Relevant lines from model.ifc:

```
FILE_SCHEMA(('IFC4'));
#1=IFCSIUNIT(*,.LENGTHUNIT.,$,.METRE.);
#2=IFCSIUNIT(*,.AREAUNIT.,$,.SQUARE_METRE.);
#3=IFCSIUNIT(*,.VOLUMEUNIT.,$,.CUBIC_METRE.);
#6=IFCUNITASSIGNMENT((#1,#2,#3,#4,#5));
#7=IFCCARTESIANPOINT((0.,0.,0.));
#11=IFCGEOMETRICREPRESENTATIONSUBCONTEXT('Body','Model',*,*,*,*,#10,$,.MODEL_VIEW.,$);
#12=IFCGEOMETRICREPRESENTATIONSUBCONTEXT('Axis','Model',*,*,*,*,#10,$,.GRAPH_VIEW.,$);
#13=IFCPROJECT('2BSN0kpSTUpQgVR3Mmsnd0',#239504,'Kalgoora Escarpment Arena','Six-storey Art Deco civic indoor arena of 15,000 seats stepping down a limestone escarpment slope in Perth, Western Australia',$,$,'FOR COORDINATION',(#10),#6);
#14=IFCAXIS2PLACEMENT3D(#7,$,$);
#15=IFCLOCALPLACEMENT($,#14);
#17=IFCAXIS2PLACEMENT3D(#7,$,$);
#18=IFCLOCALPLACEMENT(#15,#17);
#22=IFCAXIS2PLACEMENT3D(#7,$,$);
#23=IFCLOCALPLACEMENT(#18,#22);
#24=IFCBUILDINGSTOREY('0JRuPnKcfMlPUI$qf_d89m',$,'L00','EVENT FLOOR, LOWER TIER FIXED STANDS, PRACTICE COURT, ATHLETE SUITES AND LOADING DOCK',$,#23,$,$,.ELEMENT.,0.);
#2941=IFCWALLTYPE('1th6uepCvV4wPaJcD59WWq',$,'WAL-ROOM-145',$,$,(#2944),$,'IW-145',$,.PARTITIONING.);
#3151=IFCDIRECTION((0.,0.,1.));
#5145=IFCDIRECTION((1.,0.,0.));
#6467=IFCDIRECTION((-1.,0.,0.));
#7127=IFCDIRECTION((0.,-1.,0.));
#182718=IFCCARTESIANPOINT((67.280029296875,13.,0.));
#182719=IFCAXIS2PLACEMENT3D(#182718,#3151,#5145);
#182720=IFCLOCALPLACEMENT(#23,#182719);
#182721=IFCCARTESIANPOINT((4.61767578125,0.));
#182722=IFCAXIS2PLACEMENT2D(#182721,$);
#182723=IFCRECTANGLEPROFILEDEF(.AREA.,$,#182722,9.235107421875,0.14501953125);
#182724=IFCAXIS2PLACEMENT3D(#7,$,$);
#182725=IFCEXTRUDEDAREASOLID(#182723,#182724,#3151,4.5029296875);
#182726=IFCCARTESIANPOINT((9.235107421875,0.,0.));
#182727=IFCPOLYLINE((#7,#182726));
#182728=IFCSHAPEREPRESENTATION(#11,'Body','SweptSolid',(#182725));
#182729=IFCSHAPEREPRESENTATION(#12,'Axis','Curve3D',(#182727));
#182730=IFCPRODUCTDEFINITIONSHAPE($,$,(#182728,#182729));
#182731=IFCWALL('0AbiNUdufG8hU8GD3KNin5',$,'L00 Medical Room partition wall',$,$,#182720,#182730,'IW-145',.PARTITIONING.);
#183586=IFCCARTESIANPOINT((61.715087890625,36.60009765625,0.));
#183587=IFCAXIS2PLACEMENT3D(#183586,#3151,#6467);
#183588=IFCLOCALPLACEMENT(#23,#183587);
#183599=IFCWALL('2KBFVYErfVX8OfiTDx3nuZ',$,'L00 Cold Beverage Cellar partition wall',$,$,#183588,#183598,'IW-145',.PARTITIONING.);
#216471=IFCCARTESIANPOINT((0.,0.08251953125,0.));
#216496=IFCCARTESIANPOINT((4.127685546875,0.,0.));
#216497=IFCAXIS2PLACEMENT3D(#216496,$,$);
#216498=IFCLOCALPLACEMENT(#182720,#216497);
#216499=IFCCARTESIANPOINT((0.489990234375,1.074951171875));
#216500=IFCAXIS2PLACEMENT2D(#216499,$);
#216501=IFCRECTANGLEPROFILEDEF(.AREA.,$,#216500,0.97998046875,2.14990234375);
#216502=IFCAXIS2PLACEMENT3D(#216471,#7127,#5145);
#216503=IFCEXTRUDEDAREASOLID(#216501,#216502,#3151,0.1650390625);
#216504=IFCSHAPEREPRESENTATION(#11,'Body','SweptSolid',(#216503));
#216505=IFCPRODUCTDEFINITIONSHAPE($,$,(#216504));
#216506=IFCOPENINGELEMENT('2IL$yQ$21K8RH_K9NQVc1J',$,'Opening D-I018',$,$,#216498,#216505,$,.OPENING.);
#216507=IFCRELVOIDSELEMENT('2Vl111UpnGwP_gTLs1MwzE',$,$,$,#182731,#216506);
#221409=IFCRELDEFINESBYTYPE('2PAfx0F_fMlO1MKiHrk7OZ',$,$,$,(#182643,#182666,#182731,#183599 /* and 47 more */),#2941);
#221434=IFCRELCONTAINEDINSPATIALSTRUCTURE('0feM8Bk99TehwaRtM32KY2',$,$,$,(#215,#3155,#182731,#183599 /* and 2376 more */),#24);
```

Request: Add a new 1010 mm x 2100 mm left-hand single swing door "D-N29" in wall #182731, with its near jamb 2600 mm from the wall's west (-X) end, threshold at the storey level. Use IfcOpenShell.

```python
import numpy as np
import ifcopenshell
import ifcopenshell.api.feature
import ifcopenshell.api.geometry
import ifcopenshell.api.root
import ifcopenshell.api.spatial
import ifcopenshell.geom
import ifcopenshell.util.element
import ifcopenshell.util.placement
import ifcopenshell.util.representation
import ifcopenshell.util.shape
import ifcopenshell.util.unit

model = ifcopenshell.open("model.ifc")
unit_scale = ifcopenshell.util.unit.calculate_unit_scale(model)
settings = ifcopenshell.geom.settings()


def volume(element):
    """Net volume in cubic metres, openings subtracted."""
    shape = ifcopenshell.geom.create_shape(settings, element)
    return ifcopenshell.util.shape.get_volume(shape.geometry)


wall = model.by_guid("0AbiNUdufG8hU8GD3KNin5")
storey = ifcopenshell.util.element.get_container(wall, ifc_class="IfcBuildingStorey")
context = ifcopenshell.util.representation.get_context(model, "Model", "Body", "MODEL_VIEW")
before = volume(wall)

width, height, from_end, sill = 1.01, 2.1, 2.6, 0.0  # metres

# The wall runs along its own X axis, and the end named is its -X end.
wall_shape = ifcopenshell.geom.create_shape(settings, wall)
x, y, z = ifcopenshell.util.shape.get_vertices(wall_shape.geometry).T
start = x.min() + from_end
face, thickness = float(y.min()), float(y.max() - y.min())
wall_matrix = ifcopenshell.util.placement.get_local_placement(wall.ObjectPlacement)
level = ifcopenshell.util.placement.get_local_placement(storey.ObjectPlacement)[2, 3]


def in_wall(x, y):
    """Placement at x, y metres in the wall's axes, at sill height."""
    matrix = wall_matrix.copy()
    matrix[:, 3] = wall_matrix @ np.array([x / unit_scale, y / unit_scale, 0.0, 1.0])
    matrix[2, 3] = level + sill / unit_scale
    return matrix


# Opening: a box that overshoots both wall faces by 50 mm.
opening = ifcopenshell.api.root.create_entity(model, ifc_class="IfcOpeningElement", predefined_type="OPENING")
box = ifcopenshell.api.geometry.add_wall_representation(
    model, context=context, length=width, height=height, thickness=thickness + 0.1
)
ifcopenshell.api.geometry.assign_representation(model, product=opening, representation=box)
ifcopenshell.api.geometry.edit_object_placement(model, product=opening, matrix=in_wall(start, face - 0.05), is_si=False)
ifcopenshell.api.feature.add_feature(model, feature=opening, element=wall)

door = ifcopenshell.api.root.create_entity(model, ifc_class="IfcDoor", name="D-N29", predefined_type="DOOR")
door.OverallWidth, door.OverallHeight = width / unit_scale, height / unit_scale
door.OperationType = "SINGLE_SWING_LEFT"
body = ifcopenshell.api.geometry.add_door_representation(
    model,
    context=context,
    overall_width=door.OverallWidth,
    overall_height=door.OverallHeight,
    operation_type="SINGLE_SWING_LEFT",
    lining_properties={"LiningDepth": thickness / unit_scale, "ThresholdDepth": thickness / unit_scale},
)
ifcopenshell.api.geometry.assign_representation(model, product=door, representation=body)
ifcopenshell.api.spatial.assign_container(model, products=[door], relating_structure=storey)
ifcopenshell.api.feature.add_filling(model, opening=opening, element=door)

# The lining spans the wall, so the door starts at the wall face.
ifcopenshell.api.geometry.edit_object_placement(model, product=door, matrix=in_wall(start, face), is_si=False)

after = volume(wall)

print(f"wall volume {before:.3f} -> {after:.3f} m3")

model.write("model-out.ifc")
```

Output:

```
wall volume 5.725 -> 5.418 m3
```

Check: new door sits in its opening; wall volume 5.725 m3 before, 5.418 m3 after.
